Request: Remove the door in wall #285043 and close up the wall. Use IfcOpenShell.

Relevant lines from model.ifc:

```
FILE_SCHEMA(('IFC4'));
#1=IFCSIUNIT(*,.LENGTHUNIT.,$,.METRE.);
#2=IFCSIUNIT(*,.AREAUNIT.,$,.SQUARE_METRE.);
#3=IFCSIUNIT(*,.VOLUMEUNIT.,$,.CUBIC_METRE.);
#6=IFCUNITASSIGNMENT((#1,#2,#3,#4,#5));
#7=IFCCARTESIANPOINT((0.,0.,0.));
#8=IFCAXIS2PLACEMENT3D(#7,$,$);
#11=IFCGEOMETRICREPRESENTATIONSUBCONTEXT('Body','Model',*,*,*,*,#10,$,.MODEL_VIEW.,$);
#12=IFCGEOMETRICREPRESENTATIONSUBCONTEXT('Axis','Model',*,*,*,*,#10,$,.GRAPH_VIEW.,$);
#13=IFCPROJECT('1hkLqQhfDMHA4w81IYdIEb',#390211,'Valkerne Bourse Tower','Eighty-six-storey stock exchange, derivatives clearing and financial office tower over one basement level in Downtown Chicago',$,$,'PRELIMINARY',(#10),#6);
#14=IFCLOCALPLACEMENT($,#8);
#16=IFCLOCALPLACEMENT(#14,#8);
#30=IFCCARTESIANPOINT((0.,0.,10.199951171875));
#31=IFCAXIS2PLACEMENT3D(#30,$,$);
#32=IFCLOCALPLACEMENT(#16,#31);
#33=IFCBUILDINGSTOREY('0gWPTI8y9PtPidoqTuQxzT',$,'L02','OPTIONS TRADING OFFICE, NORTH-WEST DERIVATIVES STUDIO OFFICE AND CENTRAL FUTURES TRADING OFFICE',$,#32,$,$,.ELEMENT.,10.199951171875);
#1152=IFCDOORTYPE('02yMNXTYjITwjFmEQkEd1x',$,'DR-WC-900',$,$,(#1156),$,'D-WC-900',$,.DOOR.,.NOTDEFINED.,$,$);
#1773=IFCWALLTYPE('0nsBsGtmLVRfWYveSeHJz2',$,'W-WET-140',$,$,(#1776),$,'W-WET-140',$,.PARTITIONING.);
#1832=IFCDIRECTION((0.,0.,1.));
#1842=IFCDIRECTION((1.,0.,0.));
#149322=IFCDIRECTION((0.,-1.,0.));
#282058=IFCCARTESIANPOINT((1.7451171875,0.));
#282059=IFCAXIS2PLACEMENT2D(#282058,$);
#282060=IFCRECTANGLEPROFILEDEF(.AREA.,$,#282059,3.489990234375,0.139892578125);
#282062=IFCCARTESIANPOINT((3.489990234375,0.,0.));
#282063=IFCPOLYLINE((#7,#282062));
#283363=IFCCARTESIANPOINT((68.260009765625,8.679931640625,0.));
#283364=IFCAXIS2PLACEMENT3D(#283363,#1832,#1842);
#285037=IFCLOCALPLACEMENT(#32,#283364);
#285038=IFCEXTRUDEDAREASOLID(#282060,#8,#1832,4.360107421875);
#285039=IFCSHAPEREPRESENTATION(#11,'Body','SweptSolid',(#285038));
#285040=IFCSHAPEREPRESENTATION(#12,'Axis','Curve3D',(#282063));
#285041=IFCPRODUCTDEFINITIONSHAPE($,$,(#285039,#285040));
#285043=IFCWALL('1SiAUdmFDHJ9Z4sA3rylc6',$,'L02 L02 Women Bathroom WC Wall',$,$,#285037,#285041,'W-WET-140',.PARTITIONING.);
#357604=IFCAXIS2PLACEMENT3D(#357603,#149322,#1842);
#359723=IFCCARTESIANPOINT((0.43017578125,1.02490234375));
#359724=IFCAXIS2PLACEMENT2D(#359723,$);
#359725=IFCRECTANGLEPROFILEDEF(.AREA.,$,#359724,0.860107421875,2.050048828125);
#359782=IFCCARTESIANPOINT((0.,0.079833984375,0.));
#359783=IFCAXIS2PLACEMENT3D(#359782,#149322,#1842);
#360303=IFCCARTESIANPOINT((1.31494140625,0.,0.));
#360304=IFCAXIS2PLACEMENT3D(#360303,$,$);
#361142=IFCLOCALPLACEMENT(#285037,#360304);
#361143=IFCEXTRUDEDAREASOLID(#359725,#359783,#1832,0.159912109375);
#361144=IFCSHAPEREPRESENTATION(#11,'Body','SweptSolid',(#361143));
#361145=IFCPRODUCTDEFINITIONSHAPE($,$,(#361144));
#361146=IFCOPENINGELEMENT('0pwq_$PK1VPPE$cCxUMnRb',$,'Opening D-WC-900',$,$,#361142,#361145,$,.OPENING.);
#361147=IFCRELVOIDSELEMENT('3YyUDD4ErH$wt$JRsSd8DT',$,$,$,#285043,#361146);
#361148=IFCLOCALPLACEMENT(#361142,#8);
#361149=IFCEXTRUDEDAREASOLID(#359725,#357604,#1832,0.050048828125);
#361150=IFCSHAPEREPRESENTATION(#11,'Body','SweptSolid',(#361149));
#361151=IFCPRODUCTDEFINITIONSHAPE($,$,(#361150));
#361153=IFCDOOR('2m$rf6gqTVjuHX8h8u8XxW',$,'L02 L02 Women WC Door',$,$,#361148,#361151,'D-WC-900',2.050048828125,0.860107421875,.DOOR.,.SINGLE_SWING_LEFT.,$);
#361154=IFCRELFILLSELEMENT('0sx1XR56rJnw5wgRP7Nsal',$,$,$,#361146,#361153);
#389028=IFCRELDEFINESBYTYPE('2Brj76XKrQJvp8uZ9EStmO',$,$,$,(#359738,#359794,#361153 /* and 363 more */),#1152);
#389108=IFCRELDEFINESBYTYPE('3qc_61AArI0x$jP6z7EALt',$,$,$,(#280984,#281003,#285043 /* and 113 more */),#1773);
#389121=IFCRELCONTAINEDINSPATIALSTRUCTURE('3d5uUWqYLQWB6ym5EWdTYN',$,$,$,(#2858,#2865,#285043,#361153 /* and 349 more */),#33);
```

```python
import ifcopenshell
import ifcopenshell.api.feature
import ifcopenshell.api.root
import ifcopenshell.geom
import ifcopenshell.util.shape

model = ifcopenshell.open("model.ifc")
settings = ifcopenshell.geom.settings()


def volume(element):
    """Net volume in cubic metres, openings subtracted."""
    shape = ifcopenshell.geom.create_shape(settings, element)
    return ifcopenshell.util.shape.get_volume(shape.geometry)


door = model.by_guid("2m$rf6gqTVjuHX8h8u8XxW")
opening = door.FillsVoids[0].RelatingOpeningElement
wall = opening.VoidsElements[0].RelatingBuildingElement
before = volume(wall)

ifcopenshell.api.root.remove_product(model, product=door)
ifcopenshell.api.feature.remove_feature(model, feature=opening)

after = volume(wall)

print(f"wall volume {before:.3f} -> {after:.3f} m3")

model.write("model_edited.ifc")
```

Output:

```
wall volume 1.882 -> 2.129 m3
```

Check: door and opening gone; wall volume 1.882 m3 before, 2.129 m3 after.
